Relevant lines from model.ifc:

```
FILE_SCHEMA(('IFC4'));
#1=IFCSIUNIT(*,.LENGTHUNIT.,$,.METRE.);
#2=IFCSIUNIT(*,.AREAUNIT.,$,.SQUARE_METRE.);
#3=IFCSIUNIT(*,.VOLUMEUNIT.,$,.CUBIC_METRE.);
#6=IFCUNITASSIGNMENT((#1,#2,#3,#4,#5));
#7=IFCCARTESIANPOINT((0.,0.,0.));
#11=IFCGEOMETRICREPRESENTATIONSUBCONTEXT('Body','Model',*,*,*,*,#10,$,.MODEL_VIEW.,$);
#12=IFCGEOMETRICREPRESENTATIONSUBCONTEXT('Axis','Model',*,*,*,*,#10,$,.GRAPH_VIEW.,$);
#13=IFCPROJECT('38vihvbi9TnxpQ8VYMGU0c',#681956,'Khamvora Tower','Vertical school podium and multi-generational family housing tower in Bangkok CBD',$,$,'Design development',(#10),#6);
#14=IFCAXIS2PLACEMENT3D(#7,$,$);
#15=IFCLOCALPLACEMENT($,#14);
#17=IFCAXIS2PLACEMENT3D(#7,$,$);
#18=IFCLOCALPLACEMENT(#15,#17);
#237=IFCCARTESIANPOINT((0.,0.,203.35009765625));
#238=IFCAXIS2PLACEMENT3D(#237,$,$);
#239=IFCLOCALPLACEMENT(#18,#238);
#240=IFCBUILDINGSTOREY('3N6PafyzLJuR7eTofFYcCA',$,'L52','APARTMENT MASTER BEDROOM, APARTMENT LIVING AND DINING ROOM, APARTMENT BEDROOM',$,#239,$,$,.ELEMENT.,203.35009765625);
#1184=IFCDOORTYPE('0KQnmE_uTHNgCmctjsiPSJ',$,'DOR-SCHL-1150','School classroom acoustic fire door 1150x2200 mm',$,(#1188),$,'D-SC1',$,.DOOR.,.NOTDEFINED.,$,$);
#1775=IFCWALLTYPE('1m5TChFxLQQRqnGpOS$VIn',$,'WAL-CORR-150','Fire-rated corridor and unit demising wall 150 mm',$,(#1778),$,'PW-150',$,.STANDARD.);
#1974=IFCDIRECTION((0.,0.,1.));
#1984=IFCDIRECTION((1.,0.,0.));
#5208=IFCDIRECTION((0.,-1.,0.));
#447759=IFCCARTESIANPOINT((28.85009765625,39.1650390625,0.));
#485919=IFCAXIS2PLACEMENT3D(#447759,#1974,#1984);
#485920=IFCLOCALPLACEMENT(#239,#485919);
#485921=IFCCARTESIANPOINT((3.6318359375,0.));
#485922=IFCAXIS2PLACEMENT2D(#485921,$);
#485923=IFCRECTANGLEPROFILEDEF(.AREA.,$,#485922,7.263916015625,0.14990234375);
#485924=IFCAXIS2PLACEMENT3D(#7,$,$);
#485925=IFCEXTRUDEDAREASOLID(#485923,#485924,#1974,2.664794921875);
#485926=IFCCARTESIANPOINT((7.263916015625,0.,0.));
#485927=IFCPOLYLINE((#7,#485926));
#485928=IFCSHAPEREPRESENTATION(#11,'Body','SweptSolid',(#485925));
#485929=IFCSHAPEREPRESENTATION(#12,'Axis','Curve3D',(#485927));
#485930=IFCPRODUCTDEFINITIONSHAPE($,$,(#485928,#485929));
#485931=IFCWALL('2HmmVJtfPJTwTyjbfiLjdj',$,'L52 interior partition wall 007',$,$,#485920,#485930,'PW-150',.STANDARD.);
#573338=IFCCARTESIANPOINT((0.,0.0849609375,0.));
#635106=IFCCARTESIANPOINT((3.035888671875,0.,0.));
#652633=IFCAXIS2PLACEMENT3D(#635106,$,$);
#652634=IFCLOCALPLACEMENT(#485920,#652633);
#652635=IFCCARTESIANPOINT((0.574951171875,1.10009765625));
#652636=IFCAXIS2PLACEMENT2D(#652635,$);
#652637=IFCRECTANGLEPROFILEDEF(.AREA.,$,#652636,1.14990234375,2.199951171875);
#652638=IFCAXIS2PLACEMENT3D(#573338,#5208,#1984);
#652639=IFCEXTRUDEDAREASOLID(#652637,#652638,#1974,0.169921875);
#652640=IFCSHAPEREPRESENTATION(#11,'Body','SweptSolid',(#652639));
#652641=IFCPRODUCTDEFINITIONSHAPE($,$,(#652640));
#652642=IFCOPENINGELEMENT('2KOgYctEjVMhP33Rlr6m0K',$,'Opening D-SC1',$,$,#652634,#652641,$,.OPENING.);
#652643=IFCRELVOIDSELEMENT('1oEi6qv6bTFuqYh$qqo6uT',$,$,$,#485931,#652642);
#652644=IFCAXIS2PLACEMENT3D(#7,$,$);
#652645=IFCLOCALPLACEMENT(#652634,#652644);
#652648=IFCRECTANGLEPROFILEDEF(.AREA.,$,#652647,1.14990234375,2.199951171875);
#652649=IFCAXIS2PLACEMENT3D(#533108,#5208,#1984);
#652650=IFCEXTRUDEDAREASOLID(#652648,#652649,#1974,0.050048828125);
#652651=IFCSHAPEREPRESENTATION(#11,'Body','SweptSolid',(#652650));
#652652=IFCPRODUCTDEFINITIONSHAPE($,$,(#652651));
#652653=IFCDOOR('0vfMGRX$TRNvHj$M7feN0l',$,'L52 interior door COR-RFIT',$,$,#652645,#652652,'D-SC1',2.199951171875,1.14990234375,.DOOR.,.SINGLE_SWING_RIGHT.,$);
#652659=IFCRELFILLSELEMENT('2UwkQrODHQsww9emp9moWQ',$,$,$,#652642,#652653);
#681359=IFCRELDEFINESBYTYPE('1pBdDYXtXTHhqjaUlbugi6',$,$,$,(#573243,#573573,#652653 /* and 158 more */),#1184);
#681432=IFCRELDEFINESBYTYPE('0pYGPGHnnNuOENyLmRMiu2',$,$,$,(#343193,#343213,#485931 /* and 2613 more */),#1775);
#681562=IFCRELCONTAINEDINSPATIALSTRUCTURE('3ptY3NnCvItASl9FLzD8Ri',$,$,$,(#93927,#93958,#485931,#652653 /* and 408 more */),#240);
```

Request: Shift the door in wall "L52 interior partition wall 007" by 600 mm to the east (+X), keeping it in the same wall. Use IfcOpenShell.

```python
import ifcopenshell
import ifcopenshell.api.geometry
import ifcopenshell.util.placement
import ifcopenshell.util.unit

model = ifcopenshell.open("model.ifc")
unit_scale = ifcopenshell.util.unit.calculate_unit_scale(model)

door = model.by_guid("0vfMGRX$TRNvHj$M7feN0l")
opening = door.FillsVoids[0].RelatingOpeningElement
wall = opening.VoidsElements[0].RelatingBuildingElement

wall_matrix = ifcopenshell.util.placement.get_local_placement(wall.ObjectPlacement)
shift = wall_matrix[:3, 0] * 0.6 / unit_scale
before = ifcopenshell.util.placement.get_local_placement(door.ObjectPlacement)[:3, 3].copy()

# The door is placed relative to its opening, so it follows when the opening moves.
matrix = ifcopenshell.util.placement.get_local_placement(opening.ObjectPlacement)
matrix[:3, 3] += shift
ifcopenshell.api.geometry.edit_object_placement(
    model, product=opening, matrix=matrix, is_si=False, should_transform_children=True
)

after = ifcopenshell.util.placement.get_local_placement(door.ObjectPlacement)[:3, 3]
print("door moved by", (after - before).round(3) + 0.0)

model.write("model-out.ifc")
```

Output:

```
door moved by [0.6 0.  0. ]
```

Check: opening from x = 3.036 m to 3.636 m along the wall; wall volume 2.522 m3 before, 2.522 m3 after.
